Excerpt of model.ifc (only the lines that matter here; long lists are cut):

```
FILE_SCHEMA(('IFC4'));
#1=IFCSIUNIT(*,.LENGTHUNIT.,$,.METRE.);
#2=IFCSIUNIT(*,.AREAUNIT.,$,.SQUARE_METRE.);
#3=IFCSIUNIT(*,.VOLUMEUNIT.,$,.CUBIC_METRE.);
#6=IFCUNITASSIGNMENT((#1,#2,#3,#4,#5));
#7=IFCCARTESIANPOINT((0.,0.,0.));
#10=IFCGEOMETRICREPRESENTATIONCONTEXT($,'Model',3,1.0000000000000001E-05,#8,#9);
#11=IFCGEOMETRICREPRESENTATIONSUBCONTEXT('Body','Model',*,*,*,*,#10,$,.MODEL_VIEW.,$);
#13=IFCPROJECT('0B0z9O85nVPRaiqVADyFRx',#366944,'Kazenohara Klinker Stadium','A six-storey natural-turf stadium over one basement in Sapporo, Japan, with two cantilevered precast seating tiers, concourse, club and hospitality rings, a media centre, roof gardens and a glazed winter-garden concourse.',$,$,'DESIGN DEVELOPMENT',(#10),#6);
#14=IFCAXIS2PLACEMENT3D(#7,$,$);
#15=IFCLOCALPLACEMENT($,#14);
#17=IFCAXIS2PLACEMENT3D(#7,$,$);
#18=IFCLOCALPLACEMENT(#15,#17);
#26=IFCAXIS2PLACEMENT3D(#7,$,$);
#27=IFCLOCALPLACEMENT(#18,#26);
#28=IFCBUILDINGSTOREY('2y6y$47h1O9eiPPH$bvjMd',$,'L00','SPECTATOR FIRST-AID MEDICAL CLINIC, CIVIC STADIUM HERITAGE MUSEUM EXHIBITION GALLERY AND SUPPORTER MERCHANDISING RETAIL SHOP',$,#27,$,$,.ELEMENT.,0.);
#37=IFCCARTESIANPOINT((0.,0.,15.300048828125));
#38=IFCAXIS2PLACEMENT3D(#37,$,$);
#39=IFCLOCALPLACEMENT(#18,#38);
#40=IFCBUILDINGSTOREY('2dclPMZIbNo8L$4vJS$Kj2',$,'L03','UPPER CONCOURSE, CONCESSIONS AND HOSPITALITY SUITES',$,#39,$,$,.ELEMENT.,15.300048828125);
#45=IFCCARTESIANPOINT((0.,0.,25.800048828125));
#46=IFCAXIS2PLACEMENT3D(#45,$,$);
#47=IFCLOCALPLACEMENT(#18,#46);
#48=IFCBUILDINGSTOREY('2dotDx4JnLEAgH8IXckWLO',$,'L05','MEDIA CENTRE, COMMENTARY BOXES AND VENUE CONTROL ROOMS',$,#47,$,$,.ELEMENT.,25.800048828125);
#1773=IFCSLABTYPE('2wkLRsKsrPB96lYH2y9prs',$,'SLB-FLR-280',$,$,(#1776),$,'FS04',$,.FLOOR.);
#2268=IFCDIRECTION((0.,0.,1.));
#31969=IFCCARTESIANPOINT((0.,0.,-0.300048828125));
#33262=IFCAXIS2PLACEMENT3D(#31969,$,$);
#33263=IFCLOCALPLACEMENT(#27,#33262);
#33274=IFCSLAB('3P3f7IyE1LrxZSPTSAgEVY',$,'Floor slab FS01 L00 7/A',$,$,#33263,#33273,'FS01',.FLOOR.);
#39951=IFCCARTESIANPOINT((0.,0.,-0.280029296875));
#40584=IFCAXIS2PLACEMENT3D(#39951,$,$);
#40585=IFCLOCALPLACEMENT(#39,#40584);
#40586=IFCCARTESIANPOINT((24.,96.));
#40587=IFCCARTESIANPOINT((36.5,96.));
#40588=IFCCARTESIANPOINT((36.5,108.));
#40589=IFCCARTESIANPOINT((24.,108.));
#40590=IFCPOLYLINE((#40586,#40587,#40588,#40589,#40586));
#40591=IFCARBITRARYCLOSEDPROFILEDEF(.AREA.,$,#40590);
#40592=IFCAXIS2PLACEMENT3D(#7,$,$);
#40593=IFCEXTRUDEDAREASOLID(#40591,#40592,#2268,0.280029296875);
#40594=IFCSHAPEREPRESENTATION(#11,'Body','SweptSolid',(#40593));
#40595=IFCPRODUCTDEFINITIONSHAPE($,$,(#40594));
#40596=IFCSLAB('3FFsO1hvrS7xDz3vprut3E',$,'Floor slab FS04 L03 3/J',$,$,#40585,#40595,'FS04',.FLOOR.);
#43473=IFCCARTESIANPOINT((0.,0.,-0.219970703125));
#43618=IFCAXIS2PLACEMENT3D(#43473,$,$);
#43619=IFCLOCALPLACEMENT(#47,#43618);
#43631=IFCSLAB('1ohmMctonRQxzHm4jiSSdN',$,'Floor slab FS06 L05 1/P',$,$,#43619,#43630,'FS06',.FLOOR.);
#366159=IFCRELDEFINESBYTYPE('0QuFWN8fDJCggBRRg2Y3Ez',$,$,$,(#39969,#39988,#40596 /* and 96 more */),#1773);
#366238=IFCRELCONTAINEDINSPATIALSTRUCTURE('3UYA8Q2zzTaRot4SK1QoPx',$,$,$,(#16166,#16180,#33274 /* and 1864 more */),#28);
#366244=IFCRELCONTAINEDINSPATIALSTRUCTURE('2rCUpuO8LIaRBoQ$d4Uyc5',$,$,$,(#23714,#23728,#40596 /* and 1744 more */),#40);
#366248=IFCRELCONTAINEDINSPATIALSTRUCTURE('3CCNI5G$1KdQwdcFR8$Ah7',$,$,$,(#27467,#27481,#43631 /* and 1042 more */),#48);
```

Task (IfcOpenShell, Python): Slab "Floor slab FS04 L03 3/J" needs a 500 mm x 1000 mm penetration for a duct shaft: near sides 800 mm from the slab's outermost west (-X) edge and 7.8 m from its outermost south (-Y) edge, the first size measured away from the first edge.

```python
import numpy as np
import ifcopenshell
import ifcopenshell.api.feature
import ifcopenshell.api.geometry
import ifcopenshell.api.root
import ifcopenshell.geom
import ifcopenshell.util.placement
import ifcopenshell.util.representation
import ifcopenshell.util.shape
import ifcopenshell.util.unit

model = ifcopenshell.open("model.ifc")
unit_scale = ifcopenshell.util.unit.calculate_unit_scale(model)
settings = ifcopenshell.geom.settings()


def volume(element):
    """Net volume in cubic metres, openings subtracted."""
    shape = ifcopenshell.geom.create_shape(settings, element)
    return ifcopenshell.util.shape.get_volume(shape.geometry)


slab = model.by_guid("3FFsO1hvrS7xDz3vprut3E")
before = volume(slab)

# Extent in the slab's own axes, in metres. The edges named are its -X and -Y sides.
slab_shape = ifcopenshell.geom.create_shape(settings, slab)
vertices = ifcopenshell.util.shape.get_vertices(slab_shape.geometry)
x_min, y_min, bottom = vertices.min(axis=0)
top = vertices[:, 2].max()

opening = ifcopenshell.api.root.create_entity(model, ifc_class="IfcOpeningElement", name="Duct shaft opening", predefined_type="OPENING")
context = ifcopenshell.util.representation.get_context(model, "Model", "Body", "MODEL_VIEW")
width, depth = 0.5, 1
outline = [(0.0, 0.0), (width, 0.0), (width, depth), (0.0, depth), (0.0, 0.0)]
# Overshoot both faces by 50 mm so the cut is clean.
shape = ifcopenshell.api.geometry.add_slab_representation(
    model, context=context, depth=top - bottom + 0.1, polyline=outline
)
ifcopenshell.api.geometry.assign_representation(model, product=opening, representation=shape)

matrix = ifcopenshell.util.placement.get_local_placement(slab.ObjectPlacement)
matrix[:, 3] = matrix @ np.append(np.array([x_min + 0.8, y_min + 7.8, bottom - 0.05]) / unit_scale, 1.0)
ifcopenshell.api.geometry.edit_object_placement(model, product=opening, matrix=matrix, is_si=False)
ifcopenshell.api.feature.add_feature(model, feature=opening, element=slab)

after = volume(slab)

print(f"slab volume {before:.3f} -> {after:.3f} m3")

model.write("model_updated.ifc")
```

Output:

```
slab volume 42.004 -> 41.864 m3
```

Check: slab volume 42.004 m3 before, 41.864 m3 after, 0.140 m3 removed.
